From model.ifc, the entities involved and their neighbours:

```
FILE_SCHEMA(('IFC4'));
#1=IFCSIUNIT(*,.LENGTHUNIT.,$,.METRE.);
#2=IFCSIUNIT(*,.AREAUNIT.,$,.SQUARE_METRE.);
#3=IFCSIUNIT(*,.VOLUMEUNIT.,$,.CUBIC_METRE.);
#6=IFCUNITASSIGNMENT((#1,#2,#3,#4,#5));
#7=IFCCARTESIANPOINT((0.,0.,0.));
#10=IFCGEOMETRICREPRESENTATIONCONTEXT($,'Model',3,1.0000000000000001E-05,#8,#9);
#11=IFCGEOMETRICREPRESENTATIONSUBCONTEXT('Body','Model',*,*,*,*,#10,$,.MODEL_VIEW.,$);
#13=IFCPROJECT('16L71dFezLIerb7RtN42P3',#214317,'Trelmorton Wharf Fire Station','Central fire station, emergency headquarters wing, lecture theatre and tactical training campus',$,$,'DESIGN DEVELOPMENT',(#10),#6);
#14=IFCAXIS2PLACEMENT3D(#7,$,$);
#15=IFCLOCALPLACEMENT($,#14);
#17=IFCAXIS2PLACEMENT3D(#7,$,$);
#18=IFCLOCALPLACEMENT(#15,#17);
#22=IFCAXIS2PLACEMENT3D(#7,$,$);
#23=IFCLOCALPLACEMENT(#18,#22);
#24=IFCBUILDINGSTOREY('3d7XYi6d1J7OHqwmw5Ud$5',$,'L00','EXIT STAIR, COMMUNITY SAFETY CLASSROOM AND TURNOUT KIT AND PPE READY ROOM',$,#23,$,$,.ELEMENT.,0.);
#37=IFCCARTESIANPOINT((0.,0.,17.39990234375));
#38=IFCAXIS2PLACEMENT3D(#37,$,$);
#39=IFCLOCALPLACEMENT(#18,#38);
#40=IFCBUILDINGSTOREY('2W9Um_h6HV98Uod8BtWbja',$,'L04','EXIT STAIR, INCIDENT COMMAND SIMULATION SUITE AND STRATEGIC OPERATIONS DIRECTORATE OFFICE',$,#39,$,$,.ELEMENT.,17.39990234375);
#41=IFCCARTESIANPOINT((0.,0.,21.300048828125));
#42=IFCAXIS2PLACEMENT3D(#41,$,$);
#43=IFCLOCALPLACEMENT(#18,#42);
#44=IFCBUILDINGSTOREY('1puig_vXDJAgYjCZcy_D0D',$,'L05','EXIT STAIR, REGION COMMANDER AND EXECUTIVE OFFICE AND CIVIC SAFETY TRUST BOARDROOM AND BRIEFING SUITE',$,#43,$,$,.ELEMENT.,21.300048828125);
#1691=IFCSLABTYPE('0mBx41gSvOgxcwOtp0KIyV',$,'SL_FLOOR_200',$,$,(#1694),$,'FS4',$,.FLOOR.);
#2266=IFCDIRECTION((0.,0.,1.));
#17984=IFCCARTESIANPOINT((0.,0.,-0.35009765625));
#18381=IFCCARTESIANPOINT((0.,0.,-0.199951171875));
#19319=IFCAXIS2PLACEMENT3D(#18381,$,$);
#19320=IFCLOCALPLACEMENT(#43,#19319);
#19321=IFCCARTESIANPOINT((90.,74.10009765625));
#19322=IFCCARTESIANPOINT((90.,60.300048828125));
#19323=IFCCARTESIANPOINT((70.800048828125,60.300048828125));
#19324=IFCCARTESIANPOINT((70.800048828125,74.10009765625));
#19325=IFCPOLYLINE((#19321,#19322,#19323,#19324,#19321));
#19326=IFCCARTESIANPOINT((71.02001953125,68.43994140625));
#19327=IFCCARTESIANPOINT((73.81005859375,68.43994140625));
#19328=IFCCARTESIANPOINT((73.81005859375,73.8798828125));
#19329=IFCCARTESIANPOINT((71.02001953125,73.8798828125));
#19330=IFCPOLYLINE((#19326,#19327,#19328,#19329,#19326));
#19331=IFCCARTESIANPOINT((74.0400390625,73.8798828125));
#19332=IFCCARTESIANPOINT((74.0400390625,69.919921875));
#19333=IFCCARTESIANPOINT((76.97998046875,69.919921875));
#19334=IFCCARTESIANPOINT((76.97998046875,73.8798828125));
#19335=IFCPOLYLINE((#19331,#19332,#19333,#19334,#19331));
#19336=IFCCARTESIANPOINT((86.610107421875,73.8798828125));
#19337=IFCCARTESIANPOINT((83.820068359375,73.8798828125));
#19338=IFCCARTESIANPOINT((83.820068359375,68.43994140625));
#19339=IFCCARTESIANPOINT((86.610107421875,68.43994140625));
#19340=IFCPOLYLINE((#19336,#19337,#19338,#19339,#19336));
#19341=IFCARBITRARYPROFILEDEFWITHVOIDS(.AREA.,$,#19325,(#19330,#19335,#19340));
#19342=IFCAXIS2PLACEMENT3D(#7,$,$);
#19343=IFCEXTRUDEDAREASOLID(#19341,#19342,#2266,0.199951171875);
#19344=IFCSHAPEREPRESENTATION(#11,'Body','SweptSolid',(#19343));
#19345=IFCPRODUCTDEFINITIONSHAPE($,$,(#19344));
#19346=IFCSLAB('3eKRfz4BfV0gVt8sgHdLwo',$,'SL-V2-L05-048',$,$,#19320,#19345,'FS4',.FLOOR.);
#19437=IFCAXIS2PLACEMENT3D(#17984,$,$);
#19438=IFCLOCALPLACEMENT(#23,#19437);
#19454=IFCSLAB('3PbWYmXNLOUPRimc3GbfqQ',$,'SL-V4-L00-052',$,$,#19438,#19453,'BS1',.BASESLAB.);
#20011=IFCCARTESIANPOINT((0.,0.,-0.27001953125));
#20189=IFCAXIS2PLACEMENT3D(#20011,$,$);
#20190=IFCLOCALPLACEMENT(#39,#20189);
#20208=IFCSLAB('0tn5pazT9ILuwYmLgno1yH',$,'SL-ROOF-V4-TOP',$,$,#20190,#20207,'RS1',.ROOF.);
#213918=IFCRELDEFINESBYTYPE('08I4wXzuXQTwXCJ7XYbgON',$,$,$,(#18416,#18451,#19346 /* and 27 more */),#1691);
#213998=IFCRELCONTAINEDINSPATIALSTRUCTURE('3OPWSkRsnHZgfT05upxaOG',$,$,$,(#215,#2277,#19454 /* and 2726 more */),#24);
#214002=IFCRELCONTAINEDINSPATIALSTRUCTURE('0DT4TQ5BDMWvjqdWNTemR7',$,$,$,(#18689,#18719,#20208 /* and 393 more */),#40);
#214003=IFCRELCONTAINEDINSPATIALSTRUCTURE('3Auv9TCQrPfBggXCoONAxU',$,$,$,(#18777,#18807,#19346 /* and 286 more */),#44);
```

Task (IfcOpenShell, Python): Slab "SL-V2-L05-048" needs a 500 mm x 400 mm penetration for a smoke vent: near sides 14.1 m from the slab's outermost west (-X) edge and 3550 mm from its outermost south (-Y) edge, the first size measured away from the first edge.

```python
import numpy as np
import ifcopenshell
import ifcopenshell.api.feature
import ifcopenshell.api.geometry
import ifcopenshell.api.root
import ifcopenshell.geom
import ifcopenshell.util.placement
import ifcopenshell.util.representation
import ifcopenshell.util.shape
import ifcopenshell.util.unit

model = ifcopenshell.open("model.ifc")
unit_scale = ifcopenshell.util.unit.calculate_unit_scale(model)
settings = ifcopenshell.geom.settings()


def volume(element):
    """Net volume in cubic metres, openings subtracted."""
    shape = ifcopenshell.geom.create_shape(settings, element)
    return ifcopenshell.util.shape.get_volume(shape.geometry)


slab = model.by_id(19346)
before = volume(slab)

# Extent in the slab's own axes, in metres. The edges named are its -X and -Y sides.
slab_shape = ifcopenshell.geom.create_shape(settings, slab)
vertices = ifcopenshell.util.shape.get_vertices(slab_shape.geometry)
x_min, y_min, bottom = vertices.min(axis=0)
top = vertices[:, 2].max()

opening = ifcopenshell.api.root.create_entity(model, ifc_class="IfcOpeningElement", name="Smoke vent opening", predefined_type="OPENING")
context = ifcopenshell.util.representation.get_context(model, "Model", "Body", "MODEL_VIEW")
width, depth = 0.5, 0.4
outline = [(0.0, 0.0), (width, 0.0), (width, depth), (0.0, depth), (0.0, 0.0)]
# Overshoot both faces by 50 mm so the cut is clean.
shape = ifcopenshell.api.geometry.add_slab_representation(
    model, context=context, depth=top - bottom + 0.1, polyline=outline
)
ifcopenshell.api.geometry.assign_representation(model, product=opening, representation=shape)

matrix = ifcopenshell.util.placement.get_local_placement(slab.ObjectPlacement)
matrix[:, 3] = matrix @ np.append(np.array([x_min + 14.1, y_min + 3.55, bottom - 0.05]) / unit_scale, 1.0)
ifcopenshell.api.geometry.edit_object_placement(model, product=opening, matrix=matrix, is_si=False)
ifcopenshell.api.feature.add_feature(model, feature=opening, element=slab)

after = volume(slab)

print(f"slab volume {before:.3f} -> {after:.3f} m3")

model.write("model_v2.ifc")
```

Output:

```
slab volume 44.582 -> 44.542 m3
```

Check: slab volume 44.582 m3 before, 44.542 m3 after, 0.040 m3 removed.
